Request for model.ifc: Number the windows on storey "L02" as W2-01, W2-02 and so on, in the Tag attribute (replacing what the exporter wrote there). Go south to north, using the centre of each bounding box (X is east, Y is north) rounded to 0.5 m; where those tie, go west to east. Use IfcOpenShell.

First a look at what the model holds.

```python
import ifcopenshell
import ifcopenshell.util.element
import ifcopenshell.util.placement

model = ifcopenshell.open("model.ifc")
print(model.schema)
storey = next(s for s in model.by_type("IfcBuildingStorey") if s.Name == "L02")
windows = [e for e in ifcopenshell.util.element.get_decomposition(storey) if e.is_a("IfcWindow")]
for e in sorted(windows, key=lambda e: e.id()):
    origin = ifcopenshell.util.placement.get_local_placement(e.ObjectPlacement)[:3, 3]
    print(e.id(), e.Tag, e.Name, origin.round(2) + 0.0, sep=" | ")
```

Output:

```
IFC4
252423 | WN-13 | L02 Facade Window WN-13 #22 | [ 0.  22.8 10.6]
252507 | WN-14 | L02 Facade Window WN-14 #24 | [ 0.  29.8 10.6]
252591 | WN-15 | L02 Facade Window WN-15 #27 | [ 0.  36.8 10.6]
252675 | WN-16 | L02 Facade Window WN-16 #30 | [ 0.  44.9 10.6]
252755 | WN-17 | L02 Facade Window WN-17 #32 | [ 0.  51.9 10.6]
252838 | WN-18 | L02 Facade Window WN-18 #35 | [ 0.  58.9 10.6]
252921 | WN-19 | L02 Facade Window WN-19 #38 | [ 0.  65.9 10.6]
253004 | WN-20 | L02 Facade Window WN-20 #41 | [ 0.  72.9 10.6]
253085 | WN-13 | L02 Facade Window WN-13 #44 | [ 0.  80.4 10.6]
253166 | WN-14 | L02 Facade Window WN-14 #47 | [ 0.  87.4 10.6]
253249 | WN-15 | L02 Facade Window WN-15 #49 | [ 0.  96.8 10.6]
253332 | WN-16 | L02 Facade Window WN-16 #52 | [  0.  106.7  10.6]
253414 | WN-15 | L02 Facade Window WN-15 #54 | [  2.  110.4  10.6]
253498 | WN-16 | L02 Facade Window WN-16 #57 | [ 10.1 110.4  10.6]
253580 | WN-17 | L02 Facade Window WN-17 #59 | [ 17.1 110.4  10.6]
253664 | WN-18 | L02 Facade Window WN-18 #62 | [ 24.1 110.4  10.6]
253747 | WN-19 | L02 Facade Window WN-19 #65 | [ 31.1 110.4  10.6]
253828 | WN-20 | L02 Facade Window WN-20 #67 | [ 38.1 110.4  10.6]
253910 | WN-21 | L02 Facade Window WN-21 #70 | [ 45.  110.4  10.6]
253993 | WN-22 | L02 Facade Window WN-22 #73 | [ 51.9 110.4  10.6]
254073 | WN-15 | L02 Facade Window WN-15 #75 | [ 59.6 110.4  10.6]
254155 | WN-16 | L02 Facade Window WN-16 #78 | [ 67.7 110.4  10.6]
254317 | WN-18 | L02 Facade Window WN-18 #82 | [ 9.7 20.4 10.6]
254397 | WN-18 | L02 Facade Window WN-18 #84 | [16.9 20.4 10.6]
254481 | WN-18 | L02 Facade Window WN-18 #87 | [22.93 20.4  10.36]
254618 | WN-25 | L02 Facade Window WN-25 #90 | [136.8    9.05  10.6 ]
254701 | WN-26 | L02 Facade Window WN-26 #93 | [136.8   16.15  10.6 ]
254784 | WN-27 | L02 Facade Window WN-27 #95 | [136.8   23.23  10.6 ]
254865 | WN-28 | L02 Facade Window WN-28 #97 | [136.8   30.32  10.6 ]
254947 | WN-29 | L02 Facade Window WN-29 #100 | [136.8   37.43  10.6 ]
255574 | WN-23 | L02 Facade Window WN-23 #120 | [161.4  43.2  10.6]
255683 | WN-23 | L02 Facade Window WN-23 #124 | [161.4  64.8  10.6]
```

```python
import ifcopenshell
import ifcopenshell.geom
import ifcopenshell.util.element
import ifcopenshell.util.shape

model = ifcopenshell.open("model.ifc")
settings = ifcopenshell.geom.settings()
settings.set("use-world-coords", True)


def centre(element):
    shape = ifcopenshell.geom.create_shape(settings, element)
    return ifcopenshell.util.shape.get_bbox_centroid(shape.geometry)


storey = next(s for s in model.by_type("IfcBuildingStorey") if s.Name == "L02")
windows = [e for e in ifcopenshell.util.element.get_decomposition(storey) if e.is_a("IfcWindow")]

# Insertion points can sit at a corner or the storey origin, so sort by the geometry (in metres).
centres = {e: centre(e) for e in windows}
windows.sort(key=lambda e: (round(centres[e][1] / 0.5), centres[e][0]))

for i, e in enumerate(windows, start=1):
    number = f"W2-{i:02d}"
    e.Tag = number
    print(e.id(), number)

model.write("model_v2.ifc")
```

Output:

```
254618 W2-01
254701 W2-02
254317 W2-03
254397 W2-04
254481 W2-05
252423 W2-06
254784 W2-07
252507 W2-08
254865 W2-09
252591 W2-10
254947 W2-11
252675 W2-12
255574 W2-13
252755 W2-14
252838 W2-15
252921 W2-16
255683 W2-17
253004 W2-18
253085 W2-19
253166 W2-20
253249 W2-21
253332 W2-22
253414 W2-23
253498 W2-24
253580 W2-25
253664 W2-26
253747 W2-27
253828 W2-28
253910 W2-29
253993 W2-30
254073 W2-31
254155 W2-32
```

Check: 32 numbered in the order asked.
